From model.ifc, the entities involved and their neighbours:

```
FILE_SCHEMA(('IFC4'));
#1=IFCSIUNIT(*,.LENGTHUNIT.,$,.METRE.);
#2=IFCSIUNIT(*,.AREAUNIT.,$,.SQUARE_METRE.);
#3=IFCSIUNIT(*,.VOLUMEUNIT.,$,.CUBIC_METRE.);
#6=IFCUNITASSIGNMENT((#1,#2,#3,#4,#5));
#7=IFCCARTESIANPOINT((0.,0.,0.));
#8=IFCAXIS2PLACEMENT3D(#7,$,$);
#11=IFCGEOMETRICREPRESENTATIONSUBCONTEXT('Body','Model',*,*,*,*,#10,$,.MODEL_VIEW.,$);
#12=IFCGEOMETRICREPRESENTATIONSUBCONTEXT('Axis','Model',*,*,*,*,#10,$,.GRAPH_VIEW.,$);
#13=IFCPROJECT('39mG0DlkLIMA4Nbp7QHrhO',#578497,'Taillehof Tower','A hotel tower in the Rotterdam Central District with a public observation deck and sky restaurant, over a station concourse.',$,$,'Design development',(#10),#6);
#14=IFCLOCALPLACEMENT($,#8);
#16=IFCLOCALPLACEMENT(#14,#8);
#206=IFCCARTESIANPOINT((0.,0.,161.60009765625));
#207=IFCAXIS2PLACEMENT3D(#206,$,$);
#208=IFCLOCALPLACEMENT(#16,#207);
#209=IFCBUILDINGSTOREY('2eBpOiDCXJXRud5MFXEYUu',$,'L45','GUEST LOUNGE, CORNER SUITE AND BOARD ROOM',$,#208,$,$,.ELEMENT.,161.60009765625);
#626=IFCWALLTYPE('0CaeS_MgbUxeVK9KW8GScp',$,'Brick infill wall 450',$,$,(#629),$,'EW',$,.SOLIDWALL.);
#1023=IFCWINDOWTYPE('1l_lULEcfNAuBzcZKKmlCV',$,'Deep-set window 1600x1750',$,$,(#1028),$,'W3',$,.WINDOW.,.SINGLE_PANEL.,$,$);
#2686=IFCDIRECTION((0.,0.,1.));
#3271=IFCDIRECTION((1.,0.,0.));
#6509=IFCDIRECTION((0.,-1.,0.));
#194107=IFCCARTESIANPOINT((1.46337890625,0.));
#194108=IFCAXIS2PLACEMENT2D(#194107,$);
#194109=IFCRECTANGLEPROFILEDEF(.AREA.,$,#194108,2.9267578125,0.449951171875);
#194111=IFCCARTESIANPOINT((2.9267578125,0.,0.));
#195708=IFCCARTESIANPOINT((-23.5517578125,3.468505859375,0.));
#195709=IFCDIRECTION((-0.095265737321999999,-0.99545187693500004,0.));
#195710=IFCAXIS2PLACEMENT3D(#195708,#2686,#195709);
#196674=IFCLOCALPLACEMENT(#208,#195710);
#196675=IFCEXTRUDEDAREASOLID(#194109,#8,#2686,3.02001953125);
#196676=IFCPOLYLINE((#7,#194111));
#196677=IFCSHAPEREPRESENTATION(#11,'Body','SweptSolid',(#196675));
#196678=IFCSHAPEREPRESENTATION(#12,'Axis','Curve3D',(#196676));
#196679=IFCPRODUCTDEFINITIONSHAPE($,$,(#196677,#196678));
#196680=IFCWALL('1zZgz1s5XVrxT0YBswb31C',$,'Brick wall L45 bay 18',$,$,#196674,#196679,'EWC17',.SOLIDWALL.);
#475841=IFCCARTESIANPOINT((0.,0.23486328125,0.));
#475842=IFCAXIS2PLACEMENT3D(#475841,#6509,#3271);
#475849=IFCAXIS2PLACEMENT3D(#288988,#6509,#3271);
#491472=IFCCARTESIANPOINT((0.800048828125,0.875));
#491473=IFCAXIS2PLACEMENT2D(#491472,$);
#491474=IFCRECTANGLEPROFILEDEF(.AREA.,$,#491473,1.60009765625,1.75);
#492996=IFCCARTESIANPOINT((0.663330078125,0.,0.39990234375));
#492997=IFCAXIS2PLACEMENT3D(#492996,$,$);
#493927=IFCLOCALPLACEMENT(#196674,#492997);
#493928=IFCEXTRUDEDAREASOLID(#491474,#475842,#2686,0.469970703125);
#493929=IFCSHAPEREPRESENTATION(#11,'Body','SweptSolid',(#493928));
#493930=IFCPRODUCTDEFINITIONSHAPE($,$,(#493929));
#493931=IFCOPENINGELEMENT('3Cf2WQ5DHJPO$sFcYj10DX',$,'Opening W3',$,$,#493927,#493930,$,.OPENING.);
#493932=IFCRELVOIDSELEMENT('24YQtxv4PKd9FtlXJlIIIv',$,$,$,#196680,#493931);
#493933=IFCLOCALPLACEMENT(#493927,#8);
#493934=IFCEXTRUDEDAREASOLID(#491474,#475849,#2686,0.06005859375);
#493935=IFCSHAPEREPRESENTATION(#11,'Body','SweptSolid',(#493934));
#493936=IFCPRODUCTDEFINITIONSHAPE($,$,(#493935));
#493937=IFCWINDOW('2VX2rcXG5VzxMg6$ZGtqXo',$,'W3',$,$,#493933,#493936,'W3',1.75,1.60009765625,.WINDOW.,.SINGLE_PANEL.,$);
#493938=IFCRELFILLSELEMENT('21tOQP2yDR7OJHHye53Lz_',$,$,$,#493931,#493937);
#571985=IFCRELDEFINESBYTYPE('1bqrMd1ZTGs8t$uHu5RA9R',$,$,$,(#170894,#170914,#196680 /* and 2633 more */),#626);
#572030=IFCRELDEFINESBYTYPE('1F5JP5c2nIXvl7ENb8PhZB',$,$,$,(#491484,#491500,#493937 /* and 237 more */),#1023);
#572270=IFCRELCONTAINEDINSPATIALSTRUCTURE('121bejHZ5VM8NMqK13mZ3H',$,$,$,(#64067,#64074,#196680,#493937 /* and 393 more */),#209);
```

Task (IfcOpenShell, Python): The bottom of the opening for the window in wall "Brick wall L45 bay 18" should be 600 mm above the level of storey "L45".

```python
import numpy as np
import ifcopenshell
import ifcopenshell.api.geometry
import ifcopenshell.geom
import ifcopenshell.util.element
import ifcopenshell.util.placement
import ifcopenshell.util.shape
import ifcopenshell.util.unit

model = ifcopenshell.open("model.ifc")
unit_scale = ifcopenshell.util.unit.calculate_unit_scale(model)

window = model.by_id(493937)
opening = window.FillsVoids[0].RelatingOpeningElement
storey = ifcopenshell.util.element.get_container(window, ifc_class="IfcBuildingStorey")
level = ifcopenshell.util.placement.get_local_placement(storey.ObjectPlacement)[2, 3]

# The opening's origin need not be at the sill, so measure its lowest point.
shape = ifcopenshell.geom.create_shape(ifcopenshell.geom.settings(), opening)
bottom = ifcopenshell.util.shape.get_shape_bottom_elevation(shape, shape.geometry) / unit_scale
dz = level + 0.6 / unit_scale - bottom

shift = np.array([0.0, 0.0, dz])
# The window is placed relative to its opening, so it follows when the opening moves.
matrix = ifcopenshell.util.placement.get_local_placement(opening.ObjectPlacement)
matrix[:3, 3] += shift
ifcopenshell.api.geometry.edit_object_placement(
    model, product=opening, matrix=matrix, is_si=False, should_transform_children=True
)

print(f"moved by {dz * unit_scale:+.3f} m")

model.write("model_v2.ifc")
```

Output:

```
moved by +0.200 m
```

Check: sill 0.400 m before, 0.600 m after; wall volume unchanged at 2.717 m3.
